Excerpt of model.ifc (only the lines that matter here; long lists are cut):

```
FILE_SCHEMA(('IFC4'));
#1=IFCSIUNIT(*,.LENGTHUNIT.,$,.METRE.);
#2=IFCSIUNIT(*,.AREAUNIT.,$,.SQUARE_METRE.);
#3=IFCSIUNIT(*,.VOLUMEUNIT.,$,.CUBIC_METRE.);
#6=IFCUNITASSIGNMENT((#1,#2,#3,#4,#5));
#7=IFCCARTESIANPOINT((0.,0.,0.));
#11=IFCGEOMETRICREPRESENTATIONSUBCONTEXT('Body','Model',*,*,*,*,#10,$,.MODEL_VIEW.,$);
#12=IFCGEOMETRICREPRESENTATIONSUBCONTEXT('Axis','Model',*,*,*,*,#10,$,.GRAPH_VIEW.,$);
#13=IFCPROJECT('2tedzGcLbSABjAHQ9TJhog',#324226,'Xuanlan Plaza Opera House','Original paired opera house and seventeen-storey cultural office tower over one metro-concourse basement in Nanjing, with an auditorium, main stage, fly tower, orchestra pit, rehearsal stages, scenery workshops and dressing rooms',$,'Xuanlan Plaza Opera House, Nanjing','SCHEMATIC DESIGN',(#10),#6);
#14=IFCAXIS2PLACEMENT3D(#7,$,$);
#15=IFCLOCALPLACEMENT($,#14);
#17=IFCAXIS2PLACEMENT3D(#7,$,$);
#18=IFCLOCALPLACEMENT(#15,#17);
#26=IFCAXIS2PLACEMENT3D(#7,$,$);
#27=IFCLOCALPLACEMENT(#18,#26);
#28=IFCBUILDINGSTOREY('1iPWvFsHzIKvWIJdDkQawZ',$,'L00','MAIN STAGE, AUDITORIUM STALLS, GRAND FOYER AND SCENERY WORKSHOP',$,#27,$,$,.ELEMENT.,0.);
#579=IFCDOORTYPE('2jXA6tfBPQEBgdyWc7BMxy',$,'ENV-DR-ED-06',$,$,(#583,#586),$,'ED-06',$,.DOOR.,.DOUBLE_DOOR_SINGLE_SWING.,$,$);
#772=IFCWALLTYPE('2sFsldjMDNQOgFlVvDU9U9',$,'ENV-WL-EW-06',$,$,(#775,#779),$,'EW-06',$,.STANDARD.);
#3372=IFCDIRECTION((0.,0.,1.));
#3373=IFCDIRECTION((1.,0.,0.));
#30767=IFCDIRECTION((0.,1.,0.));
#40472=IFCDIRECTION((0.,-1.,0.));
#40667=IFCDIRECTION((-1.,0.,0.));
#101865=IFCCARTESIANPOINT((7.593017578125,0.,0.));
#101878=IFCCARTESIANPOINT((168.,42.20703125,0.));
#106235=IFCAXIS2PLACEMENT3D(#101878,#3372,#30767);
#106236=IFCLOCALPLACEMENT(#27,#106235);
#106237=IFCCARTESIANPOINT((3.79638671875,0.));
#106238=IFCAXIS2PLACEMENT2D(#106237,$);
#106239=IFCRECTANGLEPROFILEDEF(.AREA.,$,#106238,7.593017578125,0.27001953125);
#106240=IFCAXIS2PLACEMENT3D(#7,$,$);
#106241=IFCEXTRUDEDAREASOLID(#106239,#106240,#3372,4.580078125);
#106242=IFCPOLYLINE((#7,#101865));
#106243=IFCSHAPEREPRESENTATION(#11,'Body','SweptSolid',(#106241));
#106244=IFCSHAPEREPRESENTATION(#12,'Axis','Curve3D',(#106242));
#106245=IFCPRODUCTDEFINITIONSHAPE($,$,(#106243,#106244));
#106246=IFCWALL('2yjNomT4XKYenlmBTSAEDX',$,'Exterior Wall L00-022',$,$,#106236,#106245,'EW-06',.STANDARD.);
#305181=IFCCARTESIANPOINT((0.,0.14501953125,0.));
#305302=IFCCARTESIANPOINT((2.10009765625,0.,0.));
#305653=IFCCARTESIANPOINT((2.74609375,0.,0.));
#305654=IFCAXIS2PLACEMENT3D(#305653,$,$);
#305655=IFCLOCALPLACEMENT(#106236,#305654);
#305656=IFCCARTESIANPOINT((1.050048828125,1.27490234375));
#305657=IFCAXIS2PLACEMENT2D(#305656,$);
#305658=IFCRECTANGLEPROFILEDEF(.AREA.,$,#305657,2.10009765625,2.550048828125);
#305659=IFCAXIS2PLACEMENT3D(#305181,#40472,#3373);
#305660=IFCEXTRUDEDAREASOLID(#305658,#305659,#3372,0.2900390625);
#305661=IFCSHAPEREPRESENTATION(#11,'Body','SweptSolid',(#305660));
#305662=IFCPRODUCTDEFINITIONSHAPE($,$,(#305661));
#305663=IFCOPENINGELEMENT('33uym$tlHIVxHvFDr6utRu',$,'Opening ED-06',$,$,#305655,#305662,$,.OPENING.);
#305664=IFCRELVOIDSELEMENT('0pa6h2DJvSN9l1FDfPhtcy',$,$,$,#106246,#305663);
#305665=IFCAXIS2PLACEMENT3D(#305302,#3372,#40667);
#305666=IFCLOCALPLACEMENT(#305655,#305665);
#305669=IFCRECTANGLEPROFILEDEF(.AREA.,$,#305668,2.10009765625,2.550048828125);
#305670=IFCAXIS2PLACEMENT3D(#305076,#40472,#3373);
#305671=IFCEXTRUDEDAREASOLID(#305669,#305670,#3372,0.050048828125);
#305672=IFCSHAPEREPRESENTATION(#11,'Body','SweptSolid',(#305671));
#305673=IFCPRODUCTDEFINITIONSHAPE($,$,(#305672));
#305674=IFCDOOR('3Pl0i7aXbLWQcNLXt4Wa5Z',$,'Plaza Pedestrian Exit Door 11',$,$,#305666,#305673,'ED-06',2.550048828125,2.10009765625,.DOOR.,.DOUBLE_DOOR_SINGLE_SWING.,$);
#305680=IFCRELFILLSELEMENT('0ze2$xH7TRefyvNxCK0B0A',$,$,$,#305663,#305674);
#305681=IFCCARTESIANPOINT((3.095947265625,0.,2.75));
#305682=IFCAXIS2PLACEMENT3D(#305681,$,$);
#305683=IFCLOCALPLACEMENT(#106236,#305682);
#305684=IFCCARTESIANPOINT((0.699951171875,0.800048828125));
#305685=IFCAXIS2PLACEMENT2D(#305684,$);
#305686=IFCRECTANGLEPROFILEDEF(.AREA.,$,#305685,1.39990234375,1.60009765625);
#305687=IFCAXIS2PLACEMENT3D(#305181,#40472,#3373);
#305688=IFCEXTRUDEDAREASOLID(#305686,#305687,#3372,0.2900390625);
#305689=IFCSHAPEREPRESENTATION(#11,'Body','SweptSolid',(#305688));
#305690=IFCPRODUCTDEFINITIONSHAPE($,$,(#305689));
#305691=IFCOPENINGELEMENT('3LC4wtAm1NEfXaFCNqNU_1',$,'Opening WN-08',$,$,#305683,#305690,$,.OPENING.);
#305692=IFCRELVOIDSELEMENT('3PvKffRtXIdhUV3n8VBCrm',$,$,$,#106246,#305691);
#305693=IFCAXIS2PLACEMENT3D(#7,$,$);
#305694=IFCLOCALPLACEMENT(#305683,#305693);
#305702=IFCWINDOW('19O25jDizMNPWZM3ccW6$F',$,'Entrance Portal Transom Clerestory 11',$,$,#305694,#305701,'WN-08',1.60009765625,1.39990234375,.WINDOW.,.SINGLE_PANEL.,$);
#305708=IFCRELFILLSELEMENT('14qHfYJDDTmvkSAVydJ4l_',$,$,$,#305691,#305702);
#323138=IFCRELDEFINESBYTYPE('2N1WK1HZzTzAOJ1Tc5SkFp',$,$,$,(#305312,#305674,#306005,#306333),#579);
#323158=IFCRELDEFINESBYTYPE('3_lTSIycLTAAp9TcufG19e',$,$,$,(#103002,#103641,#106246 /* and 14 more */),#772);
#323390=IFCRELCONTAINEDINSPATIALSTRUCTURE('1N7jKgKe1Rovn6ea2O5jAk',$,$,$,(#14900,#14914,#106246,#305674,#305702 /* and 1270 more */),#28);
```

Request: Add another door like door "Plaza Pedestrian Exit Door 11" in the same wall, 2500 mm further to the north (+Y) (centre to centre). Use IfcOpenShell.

```python
import ifcopenshell
import ifcopenshell.api.feature
import ifcopenshell.api.geometry
import ifcopenshell.api.root
import ifcopenshell.geom
import ifcopenshell.util.element
import ifcopenshell.util.placement
import ifcopenshell.util.shape

model = ifcopenshell.open("model.ifc")
settings = ifcopenshell.geom.settings()


def volume(element):
    """Net volume in cubic metres, openings subtracted."""
    shape = ifcopenshell.geom.create_shape(settings, element)
    return ifcopenshell.util.shape.get_volume(shape.geometry)


door = model.by_guid("3Pl0i7aXbLWQcNLXt4Wa5Z")
opening = door.FillsVoids[0].RelatingOpeningElement
wall = opening.VoidsElements[0].RelatingBuildingElement
before = volume(wall)
shift = ifcopenshell.util.placement.get_local_placement(wall.ObjectPlacement)[:3, 0] * 2.5

# copy_class copies the void relationship, type, container and properties, but no geometry.
new_opening = ifcopenshell.api.root.copy_class(model, product=opening)
new_opening.Representation = ifcopenshell.util.element.copy_deep(
    model, opening.Representation, exclude=["IfcGeometricRepresentationContext", "IfcRepresentationMap"]
)
new_door = ifcopenshell.api.root.copy_class(model, product=door)
new_door.Representation = ifcopenshell.util.element.copy_deep(
    model, door.Representation, exclude=["IfcGeometricRepresentationContext", "IfcRepresentationMap"]
)
new_door.Tag = None
ifcopenshell.api.feature.add_filling(model, opening=new_opening, element=new_door)

for old, new in ((opening, new_opening), (door, new_door)):
    matrix = ifcopenshell.util.placement.get_local_placement(old.ObjectPlacement)
    matrix[:3, 3] += shift
    ifcopenshell.api.geometry.edit_object_placement(model, product=new, matrix=matrix, is_si=False)

after = volume(wall)

print(f"wall volume {before:.3f} -> {after:.3f} m3")

model.write("model_updated.ifc")
```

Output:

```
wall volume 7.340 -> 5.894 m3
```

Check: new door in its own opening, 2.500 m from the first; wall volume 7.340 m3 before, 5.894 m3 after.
